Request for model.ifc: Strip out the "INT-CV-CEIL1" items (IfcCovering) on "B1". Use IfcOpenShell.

First a look at what the model holds.

```python
import ifcopenshell
import ifcopenshell.util.element

model = ifcopenshell.open("model.ifc")
print(model.schema)
storey = next(s for s in model.by_type("IfcBuildingStorey") if s.Name == "B1")
coverings = [e for e in ifcopenshell.util.element.get_decomposition(storey) if e.is_a("IfcCovering")]
seen = {}
for e in coverings:
    element_type = ifcopenshell.util.element.get_type(e)
    name = element_type.Name if element_type not in (None, e) else None
    seen[name] = seen.get(name, 0) + 1
for name, count in sorted(seen.items(), key=str):
    print(count, "x", name)
```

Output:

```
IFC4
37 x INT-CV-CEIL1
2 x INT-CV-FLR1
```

```python
import ifcopenshell
import ifcopenshell.api.root
import ifcopenshell.util.element

model = ifcopenshell.open("model.ifc")

storey = next(s for s in model.by_type("IfcBuildingStorey") if s.Name == "B1")
coverings = [e for e in ifcopenshell.util.element.get_decomposition(storey) if e.is_a("IfcCovering")]
targets = [e for e in coverings if (t := ifcopenshell.util.element.get_type(e)) not in (None, e) and t.Name == "INT-CV-CEIL1"]

for e in targets:
    ifcopenshell.api.root.remove_product(model, product=e)
print(len(targets), "removed")

model.write("model_v2.ifc")
```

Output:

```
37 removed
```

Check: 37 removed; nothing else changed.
